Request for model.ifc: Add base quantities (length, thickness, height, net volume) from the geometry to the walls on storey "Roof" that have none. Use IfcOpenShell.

First a look at what the model holds.

```python
import ifcopenshell
import ifcopenshell.util.element
import ifcopenshell.util.unit

model = ifcopenshell.open("model.ifc")
print(model.schema)
for unit_type in ("LENGTHUNIT", "AREAUNIT", "VOLUMEUNIT"):
    print(unit_type, ifcopenshell.util.unit.calculate_unit_scale(model, unit_type))
storey = next(s for s in model.by_type("IfcBuildingStorey") if s.Name == "Roof")
walls = [e for e in ifcopenshell.util.element.get_decomposition(storey) if e.is_a("IfcWall")]
for e in sorted(walls, key=lambda e: e.id()):
    print(e.id(), e.is_a(), e.Name, list(ifcopenshell.util.element.get_psets(e, qtos_only=True)), sep=" | ")
```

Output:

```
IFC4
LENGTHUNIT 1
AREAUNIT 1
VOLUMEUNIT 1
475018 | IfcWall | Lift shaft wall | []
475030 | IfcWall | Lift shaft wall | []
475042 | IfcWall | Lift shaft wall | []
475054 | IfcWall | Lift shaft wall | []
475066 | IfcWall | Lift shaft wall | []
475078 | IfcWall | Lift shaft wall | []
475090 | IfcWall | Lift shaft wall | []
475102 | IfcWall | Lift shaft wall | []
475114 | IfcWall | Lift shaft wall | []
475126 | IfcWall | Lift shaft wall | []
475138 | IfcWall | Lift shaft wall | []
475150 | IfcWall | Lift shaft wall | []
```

```python
import ifcopenshell
import ifcopenshell.api.pset
import ifcopenshell.geom
import ifcopenshell.util.element
import ifcopenshell.util.shape
import ifcopenshell.util.unit

model = ifcopenshell.open("model.ifc")
unit_scale = ifcopenshell.util.unit.calculate_unit_scale(model)
volume_scale = ifcopenshell.util.unit.calculate_unit_scale(model, "VOLUMEUNIT")
settings = ifcopenshell.geom.settings()

storey = next(s for s in model.by_type("IfcBuildingStorey") if s.Name == "Roof")
walls = [e for e in ifcopenshell.util.element.get_decomposition(storey) if e.is_a("IfcWall")]

for e in sorted(walls, key=lambda e: e.id()):
    if ifcopenshell.util.element.get_psets(e, qtos_only=True, should_inherit=False):
        continue
    # Geometry comes back in metres, in the element's own axes.
    shape = ifcopenshell.geom.create_shape(settings, e)
    values = {
        "Length": ifcopenshell.util.shape.get_x(shape.geometry) / unit_scale,
        "Width": ifcopenshell.util.shape.get_y(shape.geometry) / unit_scale,
        "Height": ifcopenshell.util.shape.get_z(shape.geometry) / unit_scale,
        "NetVolume": ifcopenshell.util.shape.get_volume(shape.geometry) / volume_scale,
    }
    qto = ifcopenshell.api.pset.add_qto(model, product=e, name="Qto_WallBaseQuantities")
    ifcopenshell.api.pset.edit_qto(model, qto=qto, properties=values)
    print(e.id(), {k: round(v, 3) for k, v in values.items()})

model.write("model_v2.ifc")
```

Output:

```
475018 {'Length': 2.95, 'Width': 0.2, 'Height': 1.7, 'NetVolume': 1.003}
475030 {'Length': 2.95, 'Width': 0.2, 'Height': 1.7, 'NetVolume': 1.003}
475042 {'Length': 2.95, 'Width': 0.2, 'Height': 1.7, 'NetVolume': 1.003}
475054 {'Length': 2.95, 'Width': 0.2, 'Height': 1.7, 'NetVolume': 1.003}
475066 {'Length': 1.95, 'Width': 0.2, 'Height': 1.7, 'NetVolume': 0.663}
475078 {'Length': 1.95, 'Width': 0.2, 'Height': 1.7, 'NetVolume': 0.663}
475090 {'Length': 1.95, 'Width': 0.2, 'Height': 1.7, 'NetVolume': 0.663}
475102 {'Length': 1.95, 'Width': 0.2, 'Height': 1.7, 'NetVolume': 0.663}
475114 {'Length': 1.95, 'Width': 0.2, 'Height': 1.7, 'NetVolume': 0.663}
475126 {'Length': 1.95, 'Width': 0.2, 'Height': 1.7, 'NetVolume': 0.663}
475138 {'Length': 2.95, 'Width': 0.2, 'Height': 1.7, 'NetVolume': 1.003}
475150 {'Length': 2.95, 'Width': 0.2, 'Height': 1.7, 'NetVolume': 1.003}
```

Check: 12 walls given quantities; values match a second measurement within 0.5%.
